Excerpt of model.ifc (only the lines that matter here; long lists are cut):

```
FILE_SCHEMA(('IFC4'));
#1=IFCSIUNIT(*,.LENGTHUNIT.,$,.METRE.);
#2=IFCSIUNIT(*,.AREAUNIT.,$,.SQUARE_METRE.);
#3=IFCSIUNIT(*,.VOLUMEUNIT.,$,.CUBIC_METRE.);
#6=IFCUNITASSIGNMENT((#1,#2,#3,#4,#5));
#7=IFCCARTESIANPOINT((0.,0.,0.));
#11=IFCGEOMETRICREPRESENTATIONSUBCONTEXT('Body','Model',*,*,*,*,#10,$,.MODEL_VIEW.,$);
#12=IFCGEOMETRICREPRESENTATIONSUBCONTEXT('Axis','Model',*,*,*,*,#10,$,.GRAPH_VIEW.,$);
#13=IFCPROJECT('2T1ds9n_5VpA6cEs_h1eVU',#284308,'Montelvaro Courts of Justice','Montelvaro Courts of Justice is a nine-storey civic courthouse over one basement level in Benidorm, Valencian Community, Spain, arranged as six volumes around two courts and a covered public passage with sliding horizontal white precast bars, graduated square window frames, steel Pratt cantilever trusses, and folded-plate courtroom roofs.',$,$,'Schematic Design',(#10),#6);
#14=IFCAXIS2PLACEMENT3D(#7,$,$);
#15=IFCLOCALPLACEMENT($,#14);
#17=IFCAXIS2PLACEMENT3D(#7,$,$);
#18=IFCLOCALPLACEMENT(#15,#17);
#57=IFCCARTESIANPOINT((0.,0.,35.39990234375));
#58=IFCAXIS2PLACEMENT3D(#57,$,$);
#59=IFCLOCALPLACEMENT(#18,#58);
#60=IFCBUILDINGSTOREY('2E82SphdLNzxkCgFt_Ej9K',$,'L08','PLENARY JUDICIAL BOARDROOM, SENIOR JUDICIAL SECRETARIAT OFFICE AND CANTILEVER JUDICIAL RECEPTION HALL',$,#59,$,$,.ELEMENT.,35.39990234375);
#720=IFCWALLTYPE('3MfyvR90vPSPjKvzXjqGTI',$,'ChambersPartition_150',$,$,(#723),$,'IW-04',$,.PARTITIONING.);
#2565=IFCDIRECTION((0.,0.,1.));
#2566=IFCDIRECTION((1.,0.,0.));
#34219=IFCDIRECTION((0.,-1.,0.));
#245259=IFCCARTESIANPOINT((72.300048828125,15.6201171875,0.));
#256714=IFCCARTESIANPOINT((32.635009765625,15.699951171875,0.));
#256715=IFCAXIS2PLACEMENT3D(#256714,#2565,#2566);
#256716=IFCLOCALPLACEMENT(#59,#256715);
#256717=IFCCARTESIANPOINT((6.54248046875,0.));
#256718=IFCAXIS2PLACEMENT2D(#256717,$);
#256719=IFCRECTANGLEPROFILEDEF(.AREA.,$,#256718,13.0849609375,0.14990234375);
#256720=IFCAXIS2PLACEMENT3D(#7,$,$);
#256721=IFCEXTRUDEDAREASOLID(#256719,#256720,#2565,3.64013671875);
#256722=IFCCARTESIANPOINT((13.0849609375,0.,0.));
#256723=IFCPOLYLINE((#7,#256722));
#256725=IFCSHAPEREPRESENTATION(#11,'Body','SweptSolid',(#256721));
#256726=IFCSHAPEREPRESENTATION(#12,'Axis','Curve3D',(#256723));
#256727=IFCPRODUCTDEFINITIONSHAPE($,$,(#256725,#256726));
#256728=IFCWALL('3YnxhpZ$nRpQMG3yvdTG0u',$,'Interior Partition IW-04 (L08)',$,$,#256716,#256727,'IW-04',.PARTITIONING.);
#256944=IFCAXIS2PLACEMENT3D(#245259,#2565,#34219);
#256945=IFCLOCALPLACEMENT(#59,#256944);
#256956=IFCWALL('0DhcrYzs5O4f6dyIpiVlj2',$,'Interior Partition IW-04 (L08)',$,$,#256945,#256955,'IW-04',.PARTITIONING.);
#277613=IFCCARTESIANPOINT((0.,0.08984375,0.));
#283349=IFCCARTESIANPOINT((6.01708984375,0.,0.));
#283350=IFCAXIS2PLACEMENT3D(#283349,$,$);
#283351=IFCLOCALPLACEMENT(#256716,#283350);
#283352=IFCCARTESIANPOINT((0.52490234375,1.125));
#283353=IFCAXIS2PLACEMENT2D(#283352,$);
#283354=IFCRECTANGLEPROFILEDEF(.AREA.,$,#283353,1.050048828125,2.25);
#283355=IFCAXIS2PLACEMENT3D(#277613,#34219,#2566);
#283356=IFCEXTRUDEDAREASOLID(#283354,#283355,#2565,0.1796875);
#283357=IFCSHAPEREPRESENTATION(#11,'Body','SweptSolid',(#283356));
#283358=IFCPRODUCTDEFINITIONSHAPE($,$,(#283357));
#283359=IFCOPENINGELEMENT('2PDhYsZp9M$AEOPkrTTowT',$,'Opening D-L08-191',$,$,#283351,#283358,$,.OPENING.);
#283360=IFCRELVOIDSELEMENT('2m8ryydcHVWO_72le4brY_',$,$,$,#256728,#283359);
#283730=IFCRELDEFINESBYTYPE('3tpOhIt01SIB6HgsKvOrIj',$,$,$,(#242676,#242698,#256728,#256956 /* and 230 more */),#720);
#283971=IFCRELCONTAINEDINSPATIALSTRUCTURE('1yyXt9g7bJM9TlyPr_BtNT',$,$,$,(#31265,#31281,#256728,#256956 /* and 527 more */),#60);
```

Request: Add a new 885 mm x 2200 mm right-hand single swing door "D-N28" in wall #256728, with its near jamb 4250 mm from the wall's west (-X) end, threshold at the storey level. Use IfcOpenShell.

```python
import numpy as np
import ifcopenshell
import ifcopenshell.api.feature
import ifcopenshell.api.geometry
import ifcopenshell.api.root
import ifcopenshell.api.spatial
import ifcopenshell.geom
import ifcopenshell.util.element
import ifcopenshell.util.placement
import ifcopenshell.util.representation
import ifcopenshell.util.shape
import ifcopenshell.util.unit

model = ifcopenshell.open("model.ifc")
unit_scale = ifcopenshell.util.unit.calculate_unit_scale(model)
settings = ifcopenshell.geom.settings()


def volume(element):
    """Net volume in cubic metres, openings subtracted."""
    shape = ifcopenshell.geom.create_shape(settings, element)
    return ifcopenshell.util.shape.get_volume(shape.geometry)


wall = model.by_guid("3YnxhpZ$nRpQMG3yvdTG0u")
storey = ifcopenshell.util.element.get_container(wall, ifc_class="IfcBuildingStorey")
context = ifcopenshell.util.representation.get_context(model, "Model", "Body", "MODEL_VIEW")
before = volume(wall)

width, height, from_end, sill = 0.885, 2.2, 4.25, 0.0  # metres

# The wall runs along its own X axis, and the end named is its -X end.
wall_shape = ifcopenshell.geom.create_shape(settings, wall)
x, y, z = ifcopenshell.util.shape.get_vertices(wall_shape.geometry).T
start = x.min() + from_end
face, thickness = float(y.min()), float(y.max() - y.min())
wall_matrix = ifcopenshell.util.placement.get_local_placement(wall.ObjectPlacement)
level = ifcopenshell.util.placement.get_local_placement(storey.ObjectPlacement)[2, 3]


def in_wall(x, y):
    """Placement at x, y metres in the wall's axes, at sill height."""
    matrix = wall_matrix.copy()
    matrix[:, 3] = wall_matrix @ np.array([x / unit_scale, y / unit_scale, 0.0, 1.0])
    matrix[2, 3] = level + sill / unit_scale
    return matrix


# Opening: a box that overshoots both wall faces by 50 mm.
opening = ifcopenshell.api.root.create_entity(model, ifc_class="IfcOpeningElement", predefined_type="OPENING")
box = ifcopenshell.api.geometry.add_wall_representation(
    model, context=context, length=width, height=height, thickness=thickness + 0.1
)
ifcopenshell.api.geometry.assign_representation(model, product=opening, representation=box)
ifcopenshell.api.geometry.edit_object_placement(model, product=opening, matrix=in_wall(start, face - 0.05), is_si=False)
ifcopenshell.api.feature.add_feature(model, feature=opening, element=wall)

door = ifcopenshell.api.root.create_entity(model, ifc_class="IfcDoor", name="D-N28", predefined_type="DOOR")
door.OverallWidth, door.OverallHeight = width / unit_scale, height / unit_scale
door.OperationType = "SINGLE_SWING_RIGHT"
body = ifcopenshell.api.geometry.add_door_representation(
    model,
    context=context,
    overall_width=door.OverallWidth,
    overall_height=door.OverallHeight,
    operation_type="SINGLE_SWING_RIGHT",
    lining_properties={"LiningDepth": thickness / unit_scale, "ThresholdDepth": thickness / unit_scale},
)
ifcopenshell.api.geometry.assign_representation(model, product=door, representation=body)
ifcopenshell.api.spatial.assign_container(model, products=[door], relating_structure=storey)
ifcopenshell.api.feature.add_filling(model, opening=opening, element=door)

# The lining spans the wall, so the door starts at the wall face.
ifcopenshell.api.geometry.edit_object_placement(model, product=door, matrix=in_wall(start, face), is_si=False)

after = volume(wall)

print(f"wall volume {before:.3f} -> {after:.3f} m3")

model.write("model_v2.ifc")
```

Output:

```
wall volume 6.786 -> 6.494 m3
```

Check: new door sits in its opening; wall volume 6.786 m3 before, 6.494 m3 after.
